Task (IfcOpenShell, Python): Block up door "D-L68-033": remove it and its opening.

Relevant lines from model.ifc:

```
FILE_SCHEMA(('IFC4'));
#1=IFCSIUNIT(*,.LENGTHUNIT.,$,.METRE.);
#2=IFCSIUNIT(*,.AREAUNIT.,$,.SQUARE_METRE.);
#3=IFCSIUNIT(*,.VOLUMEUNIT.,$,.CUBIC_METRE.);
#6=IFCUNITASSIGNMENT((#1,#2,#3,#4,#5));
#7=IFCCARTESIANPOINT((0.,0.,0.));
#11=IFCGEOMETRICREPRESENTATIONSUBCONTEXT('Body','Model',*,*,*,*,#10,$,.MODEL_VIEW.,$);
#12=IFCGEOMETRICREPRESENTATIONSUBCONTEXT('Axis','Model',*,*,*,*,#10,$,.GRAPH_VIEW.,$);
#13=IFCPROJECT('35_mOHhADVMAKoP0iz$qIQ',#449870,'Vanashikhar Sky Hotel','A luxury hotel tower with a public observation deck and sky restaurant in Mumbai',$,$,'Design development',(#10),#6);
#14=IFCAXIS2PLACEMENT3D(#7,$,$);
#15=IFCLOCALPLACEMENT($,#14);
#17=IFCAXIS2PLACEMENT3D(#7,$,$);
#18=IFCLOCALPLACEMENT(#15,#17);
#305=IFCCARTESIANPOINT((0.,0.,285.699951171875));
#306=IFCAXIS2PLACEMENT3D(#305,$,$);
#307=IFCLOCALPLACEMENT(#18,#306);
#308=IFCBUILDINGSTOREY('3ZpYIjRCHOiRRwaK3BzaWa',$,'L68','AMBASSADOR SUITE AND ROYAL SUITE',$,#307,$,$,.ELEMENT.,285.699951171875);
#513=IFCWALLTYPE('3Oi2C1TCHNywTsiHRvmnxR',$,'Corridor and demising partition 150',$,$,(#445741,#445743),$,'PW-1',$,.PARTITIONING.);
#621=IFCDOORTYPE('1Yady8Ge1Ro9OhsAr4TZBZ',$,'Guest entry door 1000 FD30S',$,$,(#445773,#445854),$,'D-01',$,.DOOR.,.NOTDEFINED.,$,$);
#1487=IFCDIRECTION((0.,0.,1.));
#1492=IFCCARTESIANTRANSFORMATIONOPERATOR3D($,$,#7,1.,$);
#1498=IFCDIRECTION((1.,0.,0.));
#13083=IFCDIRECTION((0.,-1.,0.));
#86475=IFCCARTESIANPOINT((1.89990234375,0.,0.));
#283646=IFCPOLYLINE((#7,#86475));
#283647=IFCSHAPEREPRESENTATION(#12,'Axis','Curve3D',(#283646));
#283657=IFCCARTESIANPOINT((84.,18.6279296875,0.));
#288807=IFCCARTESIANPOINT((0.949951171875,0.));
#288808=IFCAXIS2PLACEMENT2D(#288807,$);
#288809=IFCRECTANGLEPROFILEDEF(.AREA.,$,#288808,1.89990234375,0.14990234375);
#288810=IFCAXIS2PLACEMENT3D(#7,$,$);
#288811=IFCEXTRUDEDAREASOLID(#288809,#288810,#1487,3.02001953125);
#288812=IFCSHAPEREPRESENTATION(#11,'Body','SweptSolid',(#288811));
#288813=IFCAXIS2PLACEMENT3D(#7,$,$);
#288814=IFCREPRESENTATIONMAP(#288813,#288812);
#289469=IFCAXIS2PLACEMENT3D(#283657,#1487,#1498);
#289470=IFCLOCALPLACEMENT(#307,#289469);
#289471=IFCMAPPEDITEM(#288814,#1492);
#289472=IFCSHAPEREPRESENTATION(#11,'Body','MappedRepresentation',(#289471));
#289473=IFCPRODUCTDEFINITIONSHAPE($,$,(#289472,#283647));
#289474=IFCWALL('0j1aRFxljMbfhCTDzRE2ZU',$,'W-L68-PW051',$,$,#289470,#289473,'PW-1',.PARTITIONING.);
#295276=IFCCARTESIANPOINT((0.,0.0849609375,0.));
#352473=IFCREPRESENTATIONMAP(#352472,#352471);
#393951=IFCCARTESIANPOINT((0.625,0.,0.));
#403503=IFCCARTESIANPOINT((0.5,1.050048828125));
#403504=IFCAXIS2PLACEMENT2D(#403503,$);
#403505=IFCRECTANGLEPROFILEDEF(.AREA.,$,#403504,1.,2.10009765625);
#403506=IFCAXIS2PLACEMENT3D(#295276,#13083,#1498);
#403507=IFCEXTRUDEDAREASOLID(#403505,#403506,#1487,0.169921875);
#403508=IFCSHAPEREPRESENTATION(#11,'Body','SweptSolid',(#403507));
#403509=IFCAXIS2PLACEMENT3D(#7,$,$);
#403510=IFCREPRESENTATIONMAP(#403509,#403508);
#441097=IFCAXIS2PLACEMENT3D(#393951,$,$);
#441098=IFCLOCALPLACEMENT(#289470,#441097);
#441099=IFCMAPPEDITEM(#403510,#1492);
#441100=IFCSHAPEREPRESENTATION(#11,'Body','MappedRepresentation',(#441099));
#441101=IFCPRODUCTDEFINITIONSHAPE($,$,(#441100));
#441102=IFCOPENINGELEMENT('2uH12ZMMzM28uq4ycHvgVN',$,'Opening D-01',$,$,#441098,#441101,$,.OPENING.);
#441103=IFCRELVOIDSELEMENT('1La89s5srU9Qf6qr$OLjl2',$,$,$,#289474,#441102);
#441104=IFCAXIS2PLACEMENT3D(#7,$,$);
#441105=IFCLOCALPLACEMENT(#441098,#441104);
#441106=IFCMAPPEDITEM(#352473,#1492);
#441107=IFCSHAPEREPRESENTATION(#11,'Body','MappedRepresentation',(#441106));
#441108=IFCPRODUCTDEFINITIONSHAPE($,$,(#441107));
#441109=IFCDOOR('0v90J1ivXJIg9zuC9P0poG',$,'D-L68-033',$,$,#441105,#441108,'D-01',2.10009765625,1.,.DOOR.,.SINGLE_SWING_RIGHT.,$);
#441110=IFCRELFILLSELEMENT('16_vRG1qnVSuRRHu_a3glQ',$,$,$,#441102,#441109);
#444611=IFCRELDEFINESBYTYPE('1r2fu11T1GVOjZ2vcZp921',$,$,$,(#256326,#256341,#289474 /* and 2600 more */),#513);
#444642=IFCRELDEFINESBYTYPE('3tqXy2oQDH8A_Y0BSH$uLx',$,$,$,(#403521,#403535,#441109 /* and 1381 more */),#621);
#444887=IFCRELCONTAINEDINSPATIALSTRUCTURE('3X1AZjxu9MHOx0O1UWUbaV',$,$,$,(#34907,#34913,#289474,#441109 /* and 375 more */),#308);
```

```python
import ifcopenshell
import ifcopenshell.api.feature
import ifcopenshell.api.root
import ifcopenshell.geom
import ifcopenshell.util.shape

model = ifcopenshell.open("model.ifc")
settings = ifcopenshell.geom.settings()


def volume(element):
    """Net volume in cubic metres, openings subtracted."""
    shape = ifcopenshell.geom.create_shape(settings, element)
    return ifcopenshell.util.shape.get_volume(shape.geometry)


door = model.by_guid("0v90J1ivXJIg9zuC9P0poG")
opening = door.FillsVoids[0].RelatingOpeningElement
wall = opening.VoidsElements[0].RelatingBuildingElement
before = volume(wall)

ifcopenshell.api.root.remove_product(model, product=door)
ifcopenshell.api.feature.remove_feature(model, feature=opening)

after = volume(wall)

print(f"wall volume {before:.3f} -> {after:.3f} m3")

model.write("model_v2.ifc")
```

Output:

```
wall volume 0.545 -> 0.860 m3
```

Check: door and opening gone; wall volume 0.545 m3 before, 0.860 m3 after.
